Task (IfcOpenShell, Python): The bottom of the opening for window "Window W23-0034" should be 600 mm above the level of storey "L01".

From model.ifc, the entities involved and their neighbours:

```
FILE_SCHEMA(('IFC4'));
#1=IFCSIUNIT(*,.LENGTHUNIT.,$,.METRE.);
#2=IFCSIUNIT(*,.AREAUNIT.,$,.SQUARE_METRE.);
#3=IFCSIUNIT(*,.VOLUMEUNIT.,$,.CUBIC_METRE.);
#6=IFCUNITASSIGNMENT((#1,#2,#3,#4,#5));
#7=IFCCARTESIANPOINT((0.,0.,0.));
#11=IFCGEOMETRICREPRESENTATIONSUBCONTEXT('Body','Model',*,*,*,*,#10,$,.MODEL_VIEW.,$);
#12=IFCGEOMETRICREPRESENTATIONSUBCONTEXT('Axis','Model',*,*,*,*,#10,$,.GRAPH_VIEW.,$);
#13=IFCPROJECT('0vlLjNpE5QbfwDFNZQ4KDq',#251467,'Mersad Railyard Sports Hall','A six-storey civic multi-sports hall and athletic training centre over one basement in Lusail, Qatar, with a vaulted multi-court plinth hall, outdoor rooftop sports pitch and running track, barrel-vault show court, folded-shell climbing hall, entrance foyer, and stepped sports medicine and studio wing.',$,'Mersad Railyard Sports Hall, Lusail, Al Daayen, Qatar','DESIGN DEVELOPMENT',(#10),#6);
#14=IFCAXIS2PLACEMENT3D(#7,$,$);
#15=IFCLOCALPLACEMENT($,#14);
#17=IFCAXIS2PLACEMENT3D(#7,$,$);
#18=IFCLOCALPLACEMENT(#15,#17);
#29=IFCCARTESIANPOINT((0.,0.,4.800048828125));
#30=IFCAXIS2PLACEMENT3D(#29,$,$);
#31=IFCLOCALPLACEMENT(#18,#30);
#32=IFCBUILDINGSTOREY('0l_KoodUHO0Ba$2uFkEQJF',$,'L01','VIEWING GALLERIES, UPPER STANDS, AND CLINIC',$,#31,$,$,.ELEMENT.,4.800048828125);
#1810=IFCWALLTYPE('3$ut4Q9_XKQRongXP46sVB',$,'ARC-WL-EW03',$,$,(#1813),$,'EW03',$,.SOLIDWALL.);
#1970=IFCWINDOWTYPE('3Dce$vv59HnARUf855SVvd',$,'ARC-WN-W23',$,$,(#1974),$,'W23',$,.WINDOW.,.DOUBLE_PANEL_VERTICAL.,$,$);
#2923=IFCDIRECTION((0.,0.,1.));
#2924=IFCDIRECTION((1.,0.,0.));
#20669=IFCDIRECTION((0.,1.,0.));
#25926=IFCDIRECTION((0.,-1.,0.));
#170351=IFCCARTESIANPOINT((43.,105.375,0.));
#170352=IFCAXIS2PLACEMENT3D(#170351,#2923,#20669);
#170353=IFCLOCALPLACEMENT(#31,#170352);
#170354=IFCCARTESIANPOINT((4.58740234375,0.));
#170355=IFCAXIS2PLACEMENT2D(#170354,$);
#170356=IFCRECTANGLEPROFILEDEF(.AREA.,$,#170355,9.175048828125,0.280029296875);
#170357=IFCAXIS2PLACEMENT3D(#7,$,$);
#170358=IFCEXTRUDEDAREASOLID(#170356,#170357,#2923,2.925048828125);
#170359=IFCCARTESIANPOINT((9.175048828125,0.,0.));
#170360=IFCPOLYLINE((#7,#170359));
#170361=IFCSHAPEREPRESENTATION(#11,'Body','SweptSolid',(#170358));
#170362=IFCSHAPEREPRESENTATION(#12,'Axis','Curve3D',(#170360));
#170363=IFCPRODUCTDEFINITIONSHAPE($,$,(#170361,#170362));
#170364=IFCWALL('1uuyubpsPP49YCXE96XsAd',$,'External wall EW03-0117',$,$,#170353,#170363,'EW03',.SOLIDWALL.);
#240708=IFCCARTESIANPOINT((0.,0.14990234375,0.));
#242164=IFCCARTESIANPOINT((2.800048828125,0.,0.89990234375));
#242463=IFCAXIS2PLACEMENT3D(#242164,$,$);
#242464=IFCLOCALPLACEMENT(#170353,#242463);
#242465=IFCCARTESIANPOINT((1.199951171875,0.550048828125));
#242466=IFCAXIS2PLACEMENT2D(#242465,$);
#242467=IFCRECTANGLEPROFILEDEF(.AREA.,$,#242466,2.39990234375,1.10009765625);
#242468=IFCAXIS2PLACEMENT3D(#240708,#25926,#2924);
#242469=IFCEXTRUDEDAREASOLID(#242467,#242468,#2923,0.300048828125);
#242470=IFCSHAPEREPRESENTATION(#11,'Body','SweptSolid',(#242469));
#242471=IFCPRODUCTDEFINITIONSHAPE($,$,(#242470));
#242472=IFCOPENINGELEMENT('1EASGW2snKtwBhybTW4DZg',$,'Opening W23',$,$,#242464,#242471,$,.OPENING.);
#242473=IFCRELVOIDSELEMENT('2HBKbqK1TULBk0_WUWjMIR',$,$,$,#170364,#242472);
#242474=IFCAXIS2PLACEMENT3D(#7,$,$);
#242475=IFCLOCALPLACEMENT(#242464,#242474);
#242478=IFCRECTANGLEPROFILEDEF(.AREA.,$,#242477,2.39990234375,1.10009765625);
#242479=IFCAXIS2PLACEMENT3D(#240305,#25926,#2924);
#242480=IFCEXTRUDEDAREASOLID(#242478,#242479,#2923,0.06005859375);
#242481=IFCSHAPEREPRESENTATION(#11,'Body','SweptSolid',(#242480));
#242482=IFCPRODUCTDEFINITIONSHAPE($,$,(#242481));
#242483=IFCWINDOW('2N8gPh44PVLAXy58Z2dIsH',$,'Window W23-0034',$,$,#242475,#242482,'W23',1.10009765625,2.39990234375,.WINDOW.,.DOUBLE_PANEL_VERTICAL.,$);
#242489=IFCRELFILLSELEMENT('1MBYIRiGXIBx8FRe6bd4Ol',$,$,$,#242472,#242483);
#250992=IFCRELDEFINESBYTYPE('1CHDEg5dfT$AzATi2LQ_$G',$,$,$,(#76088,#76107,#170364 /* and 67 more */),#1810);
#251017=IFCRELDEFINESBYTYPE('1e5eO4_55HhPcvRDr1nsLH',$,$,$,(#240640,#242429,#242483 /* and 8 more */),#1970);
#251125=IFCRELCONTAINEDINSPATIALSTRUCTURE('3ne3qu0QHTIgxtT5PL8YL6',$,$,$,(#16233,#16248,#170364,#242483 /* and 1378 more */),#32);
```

```python
import numpy as np
import ifcopenshell
import ifcopenshell.api.geometry
import ifcopenshell.geom
import ifcopenshell.util.element
import ifcopenshell.util.placement
import ifcopenshell.util.shape
import ifcopenshell.util.unit

model = ifcopenshell.open("model.ifc")
unit_scale = ifcopenshell.util.unit.calculate_unit_scale(model)

window = model.by_guid("2N8gPh44PVLAXy58Z2dIsH")
opening = window.FillsVoids[0].RelatingOpeningElement
storey = ifcopenshell.util.element.get_container(window, ifc_class="IfcBuildingStorey")
level = ifcopenshell.util.placement.get_local_placement(storey.ObjectPlacement)[2, 3]

# The opening's origin need not be at the sill, so measure its lowest point.
shape = ifcopenshell.geom.create_shape(ifcopenshell.geom.settings(), opening)
bottom = ifcopenshell.util.shape.get_shape_bottom_elevation(shape, shape.geometry) / unit_scale
dz = level + 0.6 / unit_scale - bottom

shift = np.array([0.0, 0.0, dz])
# The window is placed relative to its opening, so it follows when the opening moves.
matrix = ifcopenshell.util.placement.get_local_placement(opening.ObjectPlacement)
matrix[:3, 3] += shift
ifcopenshell.api.geometry.edit_object_placement(
    model, product=opening, matrix=matrix, is_si=False, should_transform_children=True
)

print(f"moved by {dz * unit_scale:+.3f} m")

model.write("model_updated.ifc")
```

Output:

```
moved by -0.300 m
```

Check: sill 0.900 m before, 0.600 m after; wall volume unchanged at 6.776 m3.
